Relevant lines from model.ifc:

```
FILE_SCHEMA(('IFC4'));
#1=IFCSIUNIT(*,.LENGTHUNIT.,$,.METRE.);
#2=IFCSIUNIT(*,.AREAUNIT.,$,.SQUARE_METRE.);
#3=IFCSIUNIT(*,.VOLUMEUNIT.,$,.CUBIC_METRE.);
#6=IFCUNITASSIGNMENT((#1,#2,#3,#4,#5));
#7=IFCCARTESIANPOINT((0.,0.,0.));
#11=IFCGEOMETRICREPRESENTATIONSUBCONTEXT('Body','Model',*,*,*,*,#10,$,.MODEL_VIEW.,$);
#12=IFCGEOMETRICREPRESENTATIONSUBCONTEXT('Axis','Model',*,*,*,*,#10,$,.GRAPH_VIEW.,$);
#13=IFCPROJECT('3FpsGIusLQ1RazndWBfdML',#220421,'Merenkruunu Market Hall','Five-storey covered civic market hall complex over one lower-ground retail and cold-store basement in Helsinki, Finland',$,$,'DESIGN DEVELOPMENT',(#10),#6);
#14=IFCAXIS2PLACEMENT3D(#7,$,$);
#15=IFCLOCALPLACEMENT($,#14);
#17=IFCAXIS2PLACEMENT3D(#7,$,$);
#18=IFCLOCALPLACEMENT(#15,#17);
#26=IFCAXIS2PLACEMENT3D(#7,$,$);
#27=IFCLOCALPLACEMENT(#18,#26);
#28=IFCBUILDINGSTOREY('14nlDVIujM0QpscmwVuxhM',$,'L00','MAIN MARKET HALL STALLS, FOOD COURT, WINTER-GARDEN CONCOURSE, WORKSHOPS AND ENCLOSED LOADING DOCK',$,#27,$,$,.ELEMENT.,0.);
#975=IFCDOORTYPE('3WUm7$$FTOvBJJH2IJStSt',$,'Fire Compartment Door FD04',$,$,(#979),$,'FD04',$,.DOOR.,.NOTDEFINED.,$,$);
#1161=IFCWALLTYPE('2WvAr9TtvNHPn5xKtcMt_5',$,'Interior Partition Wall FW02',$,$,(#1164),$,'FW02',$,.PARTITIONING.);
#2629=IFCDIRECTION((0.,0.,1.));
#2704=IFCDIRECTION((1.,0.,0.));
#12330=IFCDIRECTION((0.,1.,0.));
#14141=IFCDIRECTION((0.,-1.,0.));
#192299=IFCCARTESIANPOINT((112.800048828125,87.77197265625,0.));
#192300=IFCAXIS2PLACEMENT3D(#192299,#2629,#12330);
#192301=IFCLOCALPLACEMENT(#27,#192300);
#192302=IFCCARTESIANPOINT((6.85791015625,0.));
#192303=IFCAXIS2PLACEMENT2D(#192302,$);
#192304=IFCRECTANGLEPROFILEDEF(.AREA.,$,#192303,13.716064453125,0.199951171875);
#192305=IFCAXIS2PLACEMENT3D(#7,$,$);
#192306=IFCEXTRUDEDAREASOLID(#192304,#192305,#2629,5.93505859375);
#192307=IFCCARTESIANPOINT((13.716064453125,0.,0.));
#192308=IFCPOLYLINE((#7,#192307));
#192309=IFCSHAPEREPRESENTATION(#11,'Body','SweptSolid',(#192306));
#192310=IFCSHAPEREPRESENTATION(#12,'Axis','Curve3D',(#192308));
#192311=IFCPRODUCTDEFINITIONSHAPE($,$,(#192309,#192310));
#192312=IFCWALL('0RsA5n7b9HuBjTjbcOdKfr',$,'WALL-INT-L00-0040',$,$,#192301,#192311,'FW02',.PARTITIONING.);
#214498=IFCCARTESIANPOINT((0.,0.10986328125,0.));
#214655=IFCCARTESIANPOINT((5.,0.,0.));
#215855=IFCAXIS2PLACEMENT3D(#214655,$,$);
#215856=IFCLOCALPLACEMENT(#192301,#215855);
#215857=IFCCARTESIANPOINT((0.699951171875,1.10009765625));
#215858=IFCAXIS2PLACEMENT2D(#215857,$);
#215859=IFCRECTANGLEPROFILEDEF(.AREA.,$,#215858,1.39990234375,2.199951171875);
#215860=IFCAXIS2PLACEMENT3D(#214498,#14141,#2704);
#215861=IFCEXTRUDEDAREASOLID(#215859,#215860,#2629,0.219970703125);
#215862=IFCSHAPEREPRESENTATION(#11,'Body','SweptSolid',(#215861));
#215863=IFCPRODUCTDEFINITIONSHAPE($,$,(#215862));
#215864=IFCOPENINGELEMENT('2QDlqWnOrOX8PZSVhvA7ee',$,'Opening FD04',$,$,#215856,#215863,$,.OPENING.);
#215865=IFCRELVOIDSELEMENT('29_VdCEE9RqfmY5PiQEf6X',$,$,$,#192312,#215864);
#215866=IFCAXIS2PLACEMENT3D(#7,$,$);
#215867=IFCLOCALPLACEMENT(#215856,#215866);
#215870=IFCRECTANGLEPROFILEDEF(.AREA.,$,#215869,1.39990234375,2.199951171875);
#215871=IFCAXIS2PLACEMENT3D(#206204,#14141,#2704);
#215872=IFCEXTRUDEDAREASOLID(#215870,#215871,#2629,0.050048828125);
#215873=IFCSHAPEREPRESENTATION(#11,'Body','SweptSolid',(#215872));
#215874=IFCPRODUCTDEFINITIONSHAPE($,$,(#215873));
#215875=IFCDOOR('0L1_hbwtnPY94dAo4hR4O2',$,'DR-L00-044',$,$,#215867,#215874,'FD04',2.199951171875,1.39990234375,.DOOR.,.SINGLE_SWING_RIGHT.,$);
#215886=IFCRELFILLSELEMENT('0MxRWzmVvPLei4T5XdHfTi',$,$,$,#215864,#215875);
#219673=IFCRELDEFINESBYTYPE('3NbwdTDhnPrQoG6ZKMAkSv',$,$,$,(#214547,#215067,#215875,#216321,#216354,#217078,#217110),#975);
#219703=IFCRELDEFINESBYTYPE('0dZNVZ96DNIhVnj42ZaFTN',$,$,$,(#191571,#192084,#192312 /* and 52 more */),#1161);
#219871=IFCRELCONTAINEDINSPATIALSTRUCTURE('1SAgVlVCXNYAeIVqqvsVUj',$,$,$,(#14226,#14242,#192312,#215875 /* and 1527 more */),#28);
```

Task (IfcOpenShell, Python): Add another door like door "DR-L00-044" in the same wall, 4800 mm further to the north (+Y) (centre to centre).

```python
import ifcopenshell
import ifcopenshell.api.feature
import ifcopenshell.api.geometry
import ifcopenshell.api.root
import ifcopenshell.geom
import ifcopenshell.util.element
import ifcopenshell.util.placement
import ifcopenshell.util.shape
import ifcopenshell.util.unit

model = ifcopenshell.open("model.ifc")
unit_scale = ifcopenshell.util.unit.calculate_unit_scale(model)
settings = ifcopenshell.geom.settings()


def volume(element):
    """Net volume in cubic metres, openings subtracted."""
    shape = ifcopenshell.geom.create_shape(settings, element)
    return ifcopenshell.util.shape.get_volume(shape.geometry)


door = model.by_guid("0L1_hbwtnPY94dAo4hR4O2")
opening = door.FillsVoids[0].RelatingOpeningElement
wall = opening.VoidsElements[0].RelatingBuildingElement
before = volume(wall)
shift = ifcopenshell.util.placement.get_local_placement(wall.ObjectPlacement)[:3, 0] * 4.8 / unit_scale

# copy_class copies the void relationship, type, container and properties, but no geometry.
new_opening = ifcopenshell.api.root.copy_class(model, product=opening)
new_opening.Representation = ifcopenshell.util.element.copy_deep(
    model, opening.Representation, exclude=["IfcGeometricRepresentationContext", "IfcRepresentationMap"]
)
new_door = ifcopenshell.api.root.copy_class(model, product=door)
new_door.Representation = ifcopenshell.util.element.copy_deep(
    model, door.Representation, exclude=["IfcGeometricRepresentationContext", "IfcRepresentationMap"]
)
new_door.Tag = None
ifcopenshell.api.feature.add_filling(model, opening=new_opening, element=new_door)

for old, new in ((opening, new_opening), (door, new_door)):
    matrix = ifcopenshell.util.placement.get_local_placement(old.ObjectPlacement)
    matrix[:3, 3] += shift
    ifcopenshell.api.geometry.edit_object_placement(model, product=new, matrix=matrix, is_si=False)

after = volume(wall)

print(f"wall volume {before:.3f} -> {after:.3f} m3")

model.write("model_v2.ifc")
```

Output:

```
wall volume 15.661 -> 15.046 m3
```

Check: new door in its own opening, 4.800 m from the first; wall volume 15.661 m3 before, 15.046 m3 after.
